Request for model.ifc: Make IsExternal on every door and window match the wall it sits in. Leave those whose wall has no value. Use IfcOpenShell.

First a look at what the model holds.

```python
import ifcopenshell
import ifcopenshell.util.element

model = ifcopenshell.open("model.ifc")
print(model.schema)
seen = {}
for e in model.by_type("IfcDoor") + model.by_type("IfcWindow"):
    if not e.FillsVoids:
        continue
    host = e.FillsVoids[0].RelatingOpeningElement.VoidsElements[0].RelatingBuildingElement
    own = ifcopenshell.util.element.get_pset(e, f"Pset_{e.is_a()[3:].removesuffix('StandardCase')}Common", "IsExternal")
    wall = ifcopenshell.util.element.get_pset(host, "Pset_WallCommon", "IsExternal")
    seen[e.is_a(), own, wall] = seen.get((e.is_a(), own, wall), 0) + 1
for (cls, own, wall), count in sorted(seen.items(), key=str):
    print(count, cls, "IsExternal:", own, "| host wall:", wall)
```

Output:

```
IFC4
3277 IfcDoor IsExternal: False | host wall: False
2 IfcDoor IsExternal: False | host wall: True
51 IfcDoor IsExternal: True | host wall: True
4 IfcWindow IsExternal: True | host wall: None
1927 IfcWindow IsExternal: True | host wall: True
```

```python
import ifcopenshell
import ifcopenshell.api.pset
import ifcopenshell.util.element

model = ifcopenshell.open("model.ifc")

count = 0
for ifc_class, pset_name in (("IfcDoor", "Pset_DoorCommon"), ("IfcWindow", "Pset_WindowCommon")):
    for e in model.by_type(ifc_class):
        if not e.FillsVoids:
            continue
        host = e.FillsVoids[0].RelatingOpeningElement.VoidsElements[0].RelatingBuildingElement
        external = ifcopenshell.util.element.get_pset(host, "Pset_WallCommon", "IsExternal")
        if external is None or ifcopenshell.util.element.get_pset(e, pset_name, "IsExternal") == external:
            continue
        found = ifcopenshell.util.element.get_pset(e, pset_name, should_inherit=False)
        if found:
            pset = model.by_id(found["id"])
            if len(ifcopenshell.util.element.get_elements_by_pset(pset)) > 1:
                pset = ifcopenshell.api.pset.unshare_pset(model, products=[e], pset=pset)[0]
        else:
            pset = ifcopenshell.api.pset.add_pset(model, product=e, name=pset_name)
        ifcopenshell.api.pset.edit_pset(model, pset=pset, properties={"IsExternal": external})
        count += 1

print(count, "updated")

model.write("model_updated.ifc")
```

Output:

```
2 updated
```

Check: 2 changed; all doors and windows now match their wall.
